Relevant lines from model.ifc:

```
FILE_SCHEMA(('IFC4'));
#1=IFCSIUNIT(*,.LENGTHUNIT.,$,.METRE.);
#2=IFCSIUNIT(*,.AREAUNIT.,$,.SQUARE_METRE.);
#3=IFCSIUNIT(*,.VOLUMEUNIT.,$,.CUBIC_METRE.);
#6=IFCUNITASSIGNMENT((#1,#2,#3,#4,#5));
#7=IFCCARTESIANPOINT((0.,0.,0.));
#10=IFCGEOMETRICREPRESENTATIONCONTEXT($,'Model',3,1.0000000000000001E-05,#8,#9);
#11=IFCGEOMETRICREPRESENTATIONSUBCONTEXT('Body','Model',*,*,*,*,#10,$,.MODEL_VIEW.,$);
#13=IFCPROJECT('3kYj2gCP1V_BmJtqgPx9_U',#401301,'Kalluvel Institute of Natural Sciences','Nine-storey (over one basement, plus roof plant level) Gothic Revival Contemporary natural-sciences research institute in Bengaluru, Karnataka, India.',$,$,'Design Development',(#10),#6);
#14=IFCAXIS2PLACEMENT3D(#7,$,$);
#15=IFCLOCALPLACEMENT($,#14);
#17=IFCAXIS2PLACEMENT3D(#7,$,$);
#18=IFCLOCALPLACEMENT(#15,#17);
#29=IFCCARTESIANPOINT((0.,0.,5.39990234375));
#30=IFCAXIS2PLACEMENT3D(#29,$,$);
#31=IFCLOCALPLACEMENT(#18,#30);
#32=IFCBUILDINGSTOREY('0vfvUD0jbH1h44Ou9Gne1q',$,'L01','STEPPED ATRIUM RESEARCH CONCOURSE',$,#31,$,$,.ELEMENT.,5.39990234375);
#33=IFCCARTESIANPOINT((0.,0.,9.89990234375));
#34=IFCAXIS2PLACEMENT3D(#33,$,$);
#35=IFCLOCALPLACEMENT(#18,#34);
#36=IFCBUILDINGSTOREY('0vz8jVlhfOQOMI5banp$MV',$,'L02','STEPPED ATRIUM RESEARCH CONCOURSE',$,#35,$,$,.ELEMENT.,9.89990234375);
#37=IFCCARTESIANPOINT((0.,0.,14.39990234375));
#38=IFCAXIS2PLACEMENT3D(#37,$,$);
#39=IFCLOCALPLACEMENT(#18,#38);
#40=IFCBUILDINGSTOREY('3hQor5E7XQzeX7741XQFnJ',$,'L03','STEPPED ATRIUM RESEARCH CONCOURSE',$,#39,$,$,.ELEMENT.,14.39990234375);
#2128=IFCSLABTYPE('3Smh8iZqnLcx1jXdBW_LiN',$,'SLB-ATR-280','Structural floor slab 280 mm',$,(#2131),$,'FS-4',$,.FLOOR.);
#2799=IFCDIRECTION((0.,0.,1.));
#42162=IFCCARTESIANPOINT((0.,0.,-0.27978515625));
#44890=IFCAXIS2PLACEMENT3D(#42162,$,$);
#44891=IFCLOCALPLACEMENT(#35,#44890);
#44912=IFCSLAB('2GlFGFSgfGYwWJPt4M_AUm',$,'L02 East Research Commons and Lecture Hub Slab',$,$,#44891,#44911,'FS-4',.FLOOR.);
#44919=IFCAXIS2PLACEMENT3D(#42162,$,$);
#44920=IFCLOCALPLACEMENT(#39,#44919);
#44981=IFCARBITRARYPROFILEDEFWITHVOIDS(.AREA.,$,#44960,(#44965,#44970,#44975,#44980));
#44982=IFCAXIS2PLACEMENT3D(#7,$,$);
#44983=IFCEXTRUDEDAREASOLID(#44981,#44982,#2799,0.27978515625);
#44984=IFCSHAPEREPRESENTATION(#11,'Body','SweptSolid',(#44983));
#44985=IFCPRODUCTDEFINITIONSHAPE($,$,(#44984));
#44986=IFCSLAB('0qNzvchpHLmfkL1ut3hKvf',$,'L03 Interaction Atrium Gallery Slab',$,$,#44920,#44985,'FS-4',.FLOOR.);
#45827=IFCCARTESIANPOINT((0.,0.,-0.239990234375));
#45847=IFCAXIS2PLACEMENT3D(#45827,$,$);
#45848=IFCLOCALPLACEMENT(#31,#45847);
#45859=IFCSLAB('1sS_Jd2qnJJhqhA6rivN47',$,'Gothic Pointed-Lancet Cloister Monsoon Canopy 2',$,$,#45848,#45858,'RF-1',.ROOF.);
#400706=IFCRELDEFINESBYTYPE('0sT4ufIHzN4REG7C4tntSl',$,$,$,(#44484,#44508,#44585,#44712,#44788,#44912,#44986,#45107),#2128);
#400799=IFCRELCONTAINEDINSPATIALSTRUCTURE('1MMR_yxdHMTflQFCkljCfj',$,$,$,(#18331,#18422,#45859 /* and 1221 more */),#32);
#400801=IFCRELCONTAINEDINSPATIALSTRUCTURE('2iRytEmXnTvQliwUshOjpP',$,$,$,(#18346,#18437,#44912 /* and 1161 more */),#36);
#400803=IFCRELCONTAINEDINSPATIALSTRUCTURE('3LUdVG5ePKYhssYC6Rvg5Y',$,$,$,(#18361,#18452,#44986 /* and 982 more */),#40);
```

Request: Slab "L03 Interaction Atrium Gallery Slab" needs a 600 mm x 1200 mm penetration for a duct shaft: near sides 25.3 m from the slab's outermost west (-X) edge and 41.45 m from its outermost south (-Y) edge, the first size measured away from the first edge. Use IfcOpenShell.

```python
import numpy as np
import ifcopenshell
import ifcopenshell.api.feature
import ifcopenshell.api.geometry
import ifcopenshell.api.root
import ifcopenshell.geom
import ifcopenshell.util.placement
import ifcopenshell.util.representation
import ifcopenshell.util.shape
import ifcopenshell.util.unit

model = ifcopenshell.open("model.ifc")
unit_scale = ifcopenshell.util.unit.calculate_unit_scale(model)
settings = ifcopenshell.geom.settings()


def volume(element):
    """Net volume in cubic metres, openings subtracted."""
    shape = ifcopenshell.geom.create_shape(settings, element)
    return ifcopenshell.util.shape.get_volume(shape.geometry)


slab = model.by_id(44986)
before = volume(slab)

# Extent in the slab's own axes, in metres. The edges named are its -X and -Y sides.
slab_shape = ifcopenshell.geom.create_shape(settings, slab)
vertices = ifcopenshell.util.shape.get_vertices(slab_shape.geometry)
x_min, y_min, bottom = vertices.min(axis=0)
top = vertices[:, 2].max()

opening = ifcopenshell.api.root.create_entity(model, ifc_class="IfcOpeningElement", name="Duct shaft opening", predefined_type="OPENING")
context = ifcopenshell.util.representation.get_context(model, "Model", "Body", "MODEL_VIEW")
width, depth = 0.6, 1.2
outline = [(0.0, 0.0), (width, 0.0), (width, depth), (0.0, depth), (0.0, 0.0)]
# Overshoot both faces by 50 mm so the cut is clean.
shape = ifcopenshell.api.geometry.add_slab_representation(
    model, context=context, depth=top - bottom + 0.1, polyline=outline
)
ifcopenshell.api.geometry.assign_representation(model, product=opening, representation=shape)

matrix = ifcopenshell.util.placement.get_local_placement(slab.ObjectPlacement)
matrix[:, 3] = matrix @ np.append(np.array([x_min + 25.3, y_min + 41.45, bottom - 0.05]) / unit_scale, 1.0)
ifcopenshell.api.geometry.edit_object_placement(model, product=opening, matrix=matrix, is_si=False)
ifcopenshell.api.feature.add_feature(model, feature=opening, element=slab)

after = volume(slab)

print(f"slab volume {before:.3f} -> {after:.3f} m3")

model.write("model_updated.ifc")
```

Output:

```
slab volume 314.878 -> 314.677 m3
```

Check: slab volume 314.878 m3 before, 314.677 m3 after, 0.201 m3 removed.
